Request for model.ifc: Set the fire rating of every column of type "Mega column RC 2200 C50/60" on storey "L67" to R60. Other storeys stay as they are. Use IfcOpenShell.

First a look at what the model holds.

```python
import ifcopenshell
import ifcopenshell.util.element

model = ifcopenshell.open("model.ifc")
print(model.schema)
storey = next(s for s in model.by_type("IfcBuildingStorey") if s.Name == "L67")
columns = [e for e in ifcopenshell.util.element.get_decomposition(storey) if e.is_a("IfcColumn")]
seen = {}
for e in columns:
    element_type = ifcopenshell.util.element.get_type(e)
    key = (element_type.Name if element_type != e and element_type else None, ifcopenshell.util.element.get_pset(e, "Pset_ColumnCommon", "FireRating"))
    seen[key] = seen.get(key, 0) + 1
for (name, value), count in sorted(seen.items(), key=str):
    print(count, "x", name, "|", value)
```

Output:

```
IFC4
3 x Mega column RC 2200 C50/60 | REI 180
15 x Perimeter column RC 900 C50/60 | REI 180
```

```python
import ifcopenshell
import ifcopenshell.api.pset
import ifcopenshell.util.element

model = ifcopenshell.open("model.ifc")

storey = next(s for s in model.by_type("IfcBuildingStorey") if s.Name == "L67")
columns = [e for e in ifcopenshell.util.element.get_decomposition(storey) if e.is_a("IfcColumn")]

count = 0
for e in columns:
    element_type = ifcopenshell.util.element.get_type(e)
    if element_type in (None, e) or element_type.Name != "Mega column RC 2200 C50/60":
        continue
    found = ifcopenshell.util.element.get_pset(e, "Pset_ColumnCommon", should_inherit=False)
    if found:
        pset = model.by_id(found["id"])
        if len(ifcopenshell.util.element.get_elements_by_pset(pset)) > 1:
            pset = ifcopenshell.api.pset.unshare_pset(model, products=[e], pset=pset)[0]
    else:
        pset = ifcopenshell.api.pset.add_pset(model, product=e, name="Pset_ColumnCommon")
    ifcopenshell.api.pset.edit_pset(model, pset=pset, properties={"FireRating": "R60"})
    count += 1

print(count, "columns updated")

model.write("model_updated.ifc")
```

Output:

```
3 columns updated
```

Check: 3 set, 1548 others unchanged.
